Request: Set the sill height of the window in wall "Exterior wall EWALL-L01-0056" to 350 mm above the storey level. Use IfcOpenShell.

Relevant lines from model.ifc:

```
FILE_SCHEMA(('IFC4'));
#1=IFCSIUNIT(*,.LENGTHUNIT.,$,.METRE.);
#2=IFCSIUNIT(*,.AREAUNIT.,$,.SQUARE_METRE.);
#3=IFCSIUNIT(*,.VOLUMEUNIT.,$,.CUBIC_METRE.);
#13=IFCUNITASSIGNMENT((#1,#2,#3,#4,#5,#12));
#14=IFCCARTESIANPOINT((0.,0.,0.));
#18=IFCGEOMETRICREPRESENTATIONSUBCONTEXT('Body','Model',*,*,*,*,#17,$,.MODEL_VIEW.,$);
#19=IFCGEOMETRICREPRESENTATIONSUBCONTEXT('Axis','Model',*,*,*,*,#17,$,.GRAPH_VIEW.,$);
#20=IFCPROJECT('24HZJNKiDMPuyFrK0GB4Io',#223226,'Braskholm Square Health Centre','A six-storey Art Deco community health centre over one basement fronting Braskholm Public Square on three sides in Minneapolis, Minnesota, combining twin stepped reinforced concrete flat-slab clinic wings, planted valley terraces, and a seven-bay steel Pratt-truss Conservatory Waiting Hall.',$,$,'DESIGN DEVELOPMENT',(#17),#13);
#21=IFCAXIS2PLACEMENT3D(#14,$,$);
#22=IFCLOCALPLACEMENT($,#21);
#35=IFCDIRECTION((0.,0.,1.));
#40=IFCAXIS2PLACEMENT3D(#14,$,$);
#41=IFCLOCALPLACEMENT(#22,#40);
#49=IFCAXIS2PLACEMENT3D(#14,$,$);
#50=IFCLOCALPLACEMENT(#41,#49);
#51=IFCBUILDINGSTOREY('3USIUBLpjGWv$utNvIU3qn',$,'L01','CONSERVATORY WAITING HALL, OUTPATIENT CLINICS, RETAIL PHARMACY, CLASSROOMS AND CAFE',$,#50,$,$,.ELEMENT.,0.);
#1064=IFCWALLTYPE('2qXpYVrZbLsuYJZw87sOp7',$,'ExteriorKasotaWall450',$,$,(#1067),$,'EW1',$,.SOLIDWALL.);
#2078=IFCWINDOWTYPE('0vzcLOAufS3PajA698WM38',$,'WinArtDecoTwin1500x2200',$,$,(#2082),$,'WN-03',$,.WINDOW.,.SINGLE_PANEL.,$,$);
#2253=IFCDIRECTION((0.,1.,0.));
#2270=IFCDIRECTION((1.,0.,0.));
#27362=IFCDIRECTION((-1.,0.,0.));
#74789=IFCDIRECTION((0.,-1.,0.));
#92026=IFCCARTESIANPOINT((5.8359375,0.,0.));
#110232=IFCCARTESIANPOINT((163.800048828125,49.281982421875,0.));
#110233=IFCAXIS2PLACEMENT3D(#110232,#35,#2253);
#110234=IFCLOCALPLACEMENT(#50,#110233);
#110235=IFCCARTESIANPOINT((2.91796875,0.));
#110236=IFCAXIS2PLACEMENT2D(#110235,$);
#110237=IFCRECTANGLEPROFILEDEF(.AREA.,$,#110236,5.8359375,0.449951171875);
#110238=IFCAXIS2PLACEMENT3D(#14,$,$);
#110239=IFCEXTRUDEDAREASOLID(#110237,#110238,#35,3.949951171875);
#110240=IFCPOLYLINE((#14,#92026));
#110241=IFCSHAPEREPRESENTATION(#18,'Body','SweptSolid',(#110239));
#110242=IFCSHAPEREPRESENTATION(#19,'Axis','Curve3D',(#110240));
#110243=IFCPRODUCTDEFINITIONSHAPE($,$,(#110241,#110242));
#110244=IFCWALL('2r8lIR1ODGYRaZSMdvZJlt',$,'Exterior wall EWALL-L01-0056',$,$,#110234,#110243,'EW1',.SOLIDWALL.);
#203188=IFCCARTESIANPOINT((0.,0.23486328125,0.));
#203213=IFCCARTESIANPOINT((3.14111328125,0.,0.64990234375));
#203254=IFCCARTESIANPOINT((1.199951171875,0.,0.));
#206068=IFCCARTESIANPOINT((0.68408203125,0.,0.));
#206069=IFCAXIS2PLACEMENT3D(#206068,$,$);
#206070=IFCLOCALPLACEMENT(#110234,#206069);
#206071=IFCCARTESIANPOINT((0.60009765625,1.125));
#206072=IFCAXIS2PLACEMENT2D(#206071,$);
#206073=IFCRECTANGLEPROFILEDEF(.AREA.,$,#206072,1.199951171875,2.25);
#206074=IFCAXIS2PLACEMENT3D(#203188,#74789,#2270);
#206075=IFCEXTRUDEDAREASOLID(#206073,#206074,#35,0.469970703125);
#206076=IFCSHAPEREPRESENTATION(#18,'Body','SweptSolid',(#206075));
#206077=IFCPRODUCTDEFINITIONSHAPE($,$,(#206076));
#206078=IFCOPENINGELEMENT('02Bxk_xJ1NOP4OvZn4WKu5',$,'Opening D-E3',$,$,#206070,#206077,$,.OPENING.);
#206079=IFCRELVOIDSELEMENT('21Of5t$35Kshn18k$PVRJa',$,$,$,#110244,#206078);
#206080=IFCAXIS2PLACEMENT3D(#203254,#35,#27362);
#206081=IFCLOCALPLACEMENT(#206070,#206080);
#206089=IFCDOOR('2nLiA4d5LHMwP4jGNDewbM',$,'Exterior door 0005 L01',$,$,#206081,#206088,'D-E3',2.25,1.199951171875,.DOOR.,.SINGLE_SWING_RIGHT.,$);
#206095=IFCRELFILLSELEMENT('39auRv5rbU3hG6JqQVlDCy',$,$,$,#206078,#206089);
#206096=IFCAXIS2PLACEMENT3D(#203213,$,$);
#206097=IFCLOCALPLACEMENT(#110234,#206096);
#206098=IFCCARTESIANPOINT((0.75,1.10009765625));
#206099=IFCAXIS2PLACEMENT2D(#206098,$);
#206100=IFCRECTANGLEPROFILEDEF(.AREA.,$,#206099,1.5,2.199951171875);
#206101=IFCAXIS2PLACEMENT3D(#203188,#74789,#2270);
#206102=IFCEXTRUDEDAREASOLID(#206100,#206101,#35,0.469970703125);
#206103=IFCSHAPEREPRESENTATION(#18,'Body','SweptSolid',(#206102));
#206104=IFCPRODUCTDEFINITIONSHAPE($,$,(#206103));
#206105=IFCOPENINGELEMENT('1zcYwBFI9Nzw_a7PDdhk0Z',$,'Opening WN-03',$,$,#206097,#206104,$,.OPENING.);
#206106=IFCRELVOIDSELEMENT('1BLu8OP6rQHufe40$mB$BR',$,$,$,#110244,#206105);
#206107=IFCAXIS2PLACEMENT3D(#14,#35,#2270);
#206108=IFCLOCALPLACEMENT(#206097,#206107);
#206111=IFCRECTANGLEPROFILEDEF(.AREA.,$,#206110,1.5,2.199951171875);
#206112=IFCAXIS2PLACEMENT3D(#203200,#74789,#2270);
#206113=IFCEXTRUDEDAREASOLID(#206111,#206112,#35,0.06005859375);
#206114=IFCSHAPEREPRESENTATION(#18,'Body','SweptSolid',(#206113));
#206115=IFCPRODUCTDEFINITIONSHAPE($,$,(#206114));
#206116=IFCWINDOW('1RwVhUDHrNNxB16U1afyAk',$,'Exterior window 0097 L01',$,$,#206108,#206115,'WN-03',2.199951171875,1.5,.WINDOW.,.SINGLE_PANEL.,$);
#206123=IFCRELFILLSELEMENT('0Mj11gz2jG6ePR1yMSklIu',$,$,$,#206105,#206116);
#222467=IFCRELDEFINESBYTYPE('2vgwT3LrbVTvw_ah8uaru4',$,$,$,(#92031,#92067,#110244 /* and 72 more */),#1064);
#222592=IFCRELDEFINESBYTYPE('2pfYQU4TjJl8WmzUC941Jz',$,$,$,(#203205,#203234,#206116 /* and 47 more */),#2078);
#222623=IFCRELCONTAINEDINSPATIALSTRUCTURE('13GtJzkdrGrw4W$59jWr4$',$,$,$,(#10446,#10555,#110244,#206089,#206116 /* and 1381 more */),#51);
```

```python
import numpy as np
import ifcopenshell
import ifcopenshell.api.geometry
import ifcopenshell.geom
import ifcopenshell.util.element
import ifcopenshell.util.placement
import ifcopenshell.util.shape
import ifcopenshell.util.unit

model = ifcopenshell.open("model.ifc")
unit_scale = ifcopenshell.util.unit.calculate_unit_scale(model)

window = model.by_id(206116)
opening = window.FillsVoids[0].RelatingOpeningElement
storey = ifcopenshell.util.element.get_container(window, ifc_class="IfcBuildingStorey")
level = ifcopenshell.util.placement.get_local_placement(storey.ObjectPlacement)[2, 3]

# The opening's origin need not be at the sill, so measure its lowest point.
shape = ifcopenshell.geom.create_shape(ifcopenshell.geom.settings(), opening)
bottom = ifcopenshell.util.shape.get_shape_bottom_elevation(shape, shape.geometry) / unit_scale
dz = level + 0.35 - bottom

shift = np.array([0.0, 0.0, dz])
# The window is placed relative to its opening, so it follows when the opening moves.
matrix = ifcopenshell.util.placement.get_local_placement(opening.ObjectPlacement)
matrix[:3, 3] += shift
ifcopenshell.api.geometry.edit_object_placement(
    model, product=opening, matrix=matrix, is_si=False, should_transform_children=True
)

print(f"moved by {dz * unit_scale:+.3f} m")

model.write("model_edited.ifc")
```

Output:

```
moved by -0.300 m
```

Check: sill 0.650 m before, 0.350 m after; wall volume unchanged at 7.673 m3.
